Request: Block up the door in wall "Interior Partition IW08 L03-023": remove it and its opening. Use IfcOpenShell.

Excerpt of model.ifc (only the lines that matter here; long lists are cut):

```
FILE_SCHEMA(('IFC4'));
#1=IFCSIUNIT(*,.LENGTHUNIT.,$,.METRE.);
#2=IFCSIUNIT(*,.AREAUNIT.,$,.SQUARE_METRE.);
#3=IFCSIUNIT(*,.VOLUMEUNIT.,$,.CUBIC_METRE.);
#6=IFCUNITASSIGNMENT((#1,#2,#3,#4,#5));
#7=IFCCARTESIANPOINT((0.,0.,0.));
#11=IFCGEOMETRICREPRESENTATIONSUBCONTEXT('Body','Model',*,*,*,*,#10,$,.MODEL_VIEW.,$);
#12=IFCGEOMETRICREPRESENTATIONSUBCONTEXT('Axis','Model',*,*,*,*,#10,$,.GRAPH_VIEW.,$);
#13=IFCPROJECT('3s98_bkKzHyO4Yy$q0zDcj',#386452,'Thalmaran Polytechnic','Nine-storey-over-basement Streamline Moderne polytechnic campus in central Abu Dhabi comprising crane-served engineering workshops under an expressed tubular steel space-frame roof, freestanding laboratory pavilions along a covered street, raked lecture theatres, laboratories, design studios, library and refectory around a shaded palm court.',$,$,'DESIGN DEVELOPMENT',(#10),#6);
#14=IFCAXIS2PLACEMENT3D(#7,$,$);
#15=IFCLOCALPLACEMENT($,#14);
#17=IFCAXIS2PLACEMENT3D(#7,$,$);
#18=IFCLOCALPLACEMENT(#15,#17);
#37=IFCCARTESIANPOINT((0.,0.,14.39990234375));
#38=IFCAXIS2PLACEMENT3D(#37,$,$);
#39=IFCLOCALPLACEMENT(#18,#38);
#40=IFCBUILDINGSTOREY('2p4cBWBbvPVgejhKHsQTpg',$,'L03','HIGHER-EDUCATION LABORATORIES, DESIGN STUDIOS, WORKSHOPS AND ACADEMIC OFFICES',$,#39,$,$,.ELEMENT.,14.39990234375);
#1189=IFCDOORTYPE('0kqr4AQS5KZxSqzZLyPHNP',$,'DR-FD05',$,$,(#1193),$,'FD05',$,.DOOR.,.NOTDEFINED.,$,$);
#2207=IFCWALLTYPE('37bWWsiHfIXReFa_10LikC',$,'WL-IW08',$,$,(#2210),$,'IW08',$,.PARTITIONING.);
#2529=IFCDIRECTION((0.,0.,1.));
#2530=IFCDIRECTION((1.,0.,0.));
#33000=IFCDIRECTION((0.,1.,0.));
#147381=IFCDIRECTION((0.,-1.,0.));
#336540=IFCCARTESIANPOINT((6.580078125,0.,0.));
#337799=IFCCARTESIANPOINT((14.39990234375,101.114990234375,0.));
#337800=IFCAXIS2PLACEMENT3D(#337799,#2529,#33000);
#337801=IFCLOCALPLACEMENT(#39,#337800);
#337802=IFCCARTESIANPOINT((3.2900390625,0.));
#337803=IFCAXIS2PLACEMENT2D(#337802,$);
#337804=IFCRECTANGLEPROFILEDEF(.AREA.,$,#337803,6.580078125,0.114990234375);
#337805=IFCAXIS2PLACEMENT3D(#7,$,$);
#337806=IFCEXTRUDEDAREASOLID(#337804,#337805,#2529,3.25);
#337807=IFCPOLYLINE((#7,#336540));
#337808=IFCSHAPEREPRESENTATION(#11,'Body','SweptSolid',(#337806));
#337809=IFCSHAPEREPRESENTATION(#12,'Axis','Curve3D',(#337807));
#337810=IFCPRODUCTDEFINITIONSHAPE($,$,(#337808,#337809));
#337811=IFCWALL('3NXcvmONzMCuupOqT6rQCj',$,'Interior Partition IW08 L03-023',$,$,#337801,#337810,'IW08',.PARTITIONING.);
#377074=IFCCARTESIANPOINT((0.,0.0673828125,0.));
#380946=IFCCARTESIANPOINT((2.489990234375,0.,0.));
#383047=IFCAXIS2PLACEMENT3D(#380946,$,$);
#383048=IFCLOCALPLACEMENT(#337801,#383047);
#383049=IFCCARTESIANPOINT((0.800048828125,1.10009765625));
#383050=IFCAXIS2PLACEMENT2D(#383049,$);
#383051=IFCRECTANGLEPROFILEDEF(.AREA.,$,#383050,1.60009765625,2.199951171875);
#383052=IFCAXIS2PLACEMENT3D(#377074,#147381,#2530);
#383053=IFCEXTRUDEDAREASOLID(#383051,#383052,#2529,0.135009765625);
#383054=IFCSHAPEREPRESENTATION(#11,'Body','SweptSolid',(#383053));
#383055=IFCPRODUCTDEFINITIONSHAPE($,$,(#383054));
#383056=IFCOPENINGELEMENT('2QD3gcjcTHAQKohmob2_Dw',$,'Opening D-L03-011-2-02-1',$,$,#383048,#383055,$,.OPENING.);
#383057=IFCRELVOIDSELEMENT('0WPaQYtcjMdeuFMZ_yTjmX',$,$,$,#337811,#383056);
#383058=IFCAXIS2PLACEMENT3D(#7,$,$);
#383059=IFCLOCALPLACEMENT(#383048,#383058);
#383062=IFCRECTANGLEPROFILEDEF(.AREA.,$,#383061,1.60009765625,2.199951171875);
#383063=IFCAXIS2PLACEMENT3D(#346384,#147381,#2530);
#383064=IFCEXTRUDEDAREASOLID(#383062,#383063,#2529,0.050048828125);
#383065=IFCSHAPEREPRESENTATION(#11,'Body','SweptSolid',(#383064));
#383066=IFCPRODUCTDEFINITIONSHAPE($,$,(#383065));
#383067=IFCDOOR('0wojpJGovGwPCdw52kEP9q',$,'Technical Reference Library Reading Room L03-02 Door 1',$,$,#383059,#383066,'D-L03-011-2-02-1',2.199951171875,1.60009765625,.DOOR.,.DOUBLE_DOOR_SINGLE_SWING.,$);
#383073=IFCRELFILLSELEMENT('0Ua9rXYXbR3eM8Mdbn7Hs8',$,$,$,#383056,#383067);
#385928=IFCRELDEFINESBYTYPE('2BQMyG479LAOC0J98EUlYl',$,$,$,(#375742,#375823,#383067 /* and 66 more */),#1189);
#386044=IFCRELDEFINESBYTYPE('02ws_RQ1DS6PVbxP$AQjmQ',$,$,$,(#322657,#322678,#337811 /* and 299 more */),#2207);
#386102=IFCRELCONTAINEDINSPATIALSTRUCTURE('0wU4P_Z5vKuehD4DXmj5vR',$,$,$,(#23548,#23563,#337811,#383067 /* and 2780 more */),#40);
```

```python
import ifcopenshell
import ifcopenshell.api.feature
import ifcopenshell.api.root
import ifcopenshell.geom
import ifcopenshell.util.shape

model = ifcopenshell.open("model.ifc")
settings = ifcopenshell.geom.settings()


def volume(element):
    """Net volume in cubic metres, openings subtracted."""
    shape = ifcopenshell.geom.create_shape(settings, element)
    return ifcopenshell.util.shape.get_volume(shape.geometry)


door = model.by_id(383067)
opening = door.FillsVoids[0].RelatingOpeningElement
wall = opening.VoidsElements[0].RelatingBuildingElement
before = volume(wall)

ifcopenshell.api.root.remove_product(model, product=door)
ifcopenshell.api.feature.remove_feature(model, feature=opening)

after = volume(wall)

print(f"wall volume {before:.3f} -> {after:.3f} m3")

model.write("model_edited.ifc")
```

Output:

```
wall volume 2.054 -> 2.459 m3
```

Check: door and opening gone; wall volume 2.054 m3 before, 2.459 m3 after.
